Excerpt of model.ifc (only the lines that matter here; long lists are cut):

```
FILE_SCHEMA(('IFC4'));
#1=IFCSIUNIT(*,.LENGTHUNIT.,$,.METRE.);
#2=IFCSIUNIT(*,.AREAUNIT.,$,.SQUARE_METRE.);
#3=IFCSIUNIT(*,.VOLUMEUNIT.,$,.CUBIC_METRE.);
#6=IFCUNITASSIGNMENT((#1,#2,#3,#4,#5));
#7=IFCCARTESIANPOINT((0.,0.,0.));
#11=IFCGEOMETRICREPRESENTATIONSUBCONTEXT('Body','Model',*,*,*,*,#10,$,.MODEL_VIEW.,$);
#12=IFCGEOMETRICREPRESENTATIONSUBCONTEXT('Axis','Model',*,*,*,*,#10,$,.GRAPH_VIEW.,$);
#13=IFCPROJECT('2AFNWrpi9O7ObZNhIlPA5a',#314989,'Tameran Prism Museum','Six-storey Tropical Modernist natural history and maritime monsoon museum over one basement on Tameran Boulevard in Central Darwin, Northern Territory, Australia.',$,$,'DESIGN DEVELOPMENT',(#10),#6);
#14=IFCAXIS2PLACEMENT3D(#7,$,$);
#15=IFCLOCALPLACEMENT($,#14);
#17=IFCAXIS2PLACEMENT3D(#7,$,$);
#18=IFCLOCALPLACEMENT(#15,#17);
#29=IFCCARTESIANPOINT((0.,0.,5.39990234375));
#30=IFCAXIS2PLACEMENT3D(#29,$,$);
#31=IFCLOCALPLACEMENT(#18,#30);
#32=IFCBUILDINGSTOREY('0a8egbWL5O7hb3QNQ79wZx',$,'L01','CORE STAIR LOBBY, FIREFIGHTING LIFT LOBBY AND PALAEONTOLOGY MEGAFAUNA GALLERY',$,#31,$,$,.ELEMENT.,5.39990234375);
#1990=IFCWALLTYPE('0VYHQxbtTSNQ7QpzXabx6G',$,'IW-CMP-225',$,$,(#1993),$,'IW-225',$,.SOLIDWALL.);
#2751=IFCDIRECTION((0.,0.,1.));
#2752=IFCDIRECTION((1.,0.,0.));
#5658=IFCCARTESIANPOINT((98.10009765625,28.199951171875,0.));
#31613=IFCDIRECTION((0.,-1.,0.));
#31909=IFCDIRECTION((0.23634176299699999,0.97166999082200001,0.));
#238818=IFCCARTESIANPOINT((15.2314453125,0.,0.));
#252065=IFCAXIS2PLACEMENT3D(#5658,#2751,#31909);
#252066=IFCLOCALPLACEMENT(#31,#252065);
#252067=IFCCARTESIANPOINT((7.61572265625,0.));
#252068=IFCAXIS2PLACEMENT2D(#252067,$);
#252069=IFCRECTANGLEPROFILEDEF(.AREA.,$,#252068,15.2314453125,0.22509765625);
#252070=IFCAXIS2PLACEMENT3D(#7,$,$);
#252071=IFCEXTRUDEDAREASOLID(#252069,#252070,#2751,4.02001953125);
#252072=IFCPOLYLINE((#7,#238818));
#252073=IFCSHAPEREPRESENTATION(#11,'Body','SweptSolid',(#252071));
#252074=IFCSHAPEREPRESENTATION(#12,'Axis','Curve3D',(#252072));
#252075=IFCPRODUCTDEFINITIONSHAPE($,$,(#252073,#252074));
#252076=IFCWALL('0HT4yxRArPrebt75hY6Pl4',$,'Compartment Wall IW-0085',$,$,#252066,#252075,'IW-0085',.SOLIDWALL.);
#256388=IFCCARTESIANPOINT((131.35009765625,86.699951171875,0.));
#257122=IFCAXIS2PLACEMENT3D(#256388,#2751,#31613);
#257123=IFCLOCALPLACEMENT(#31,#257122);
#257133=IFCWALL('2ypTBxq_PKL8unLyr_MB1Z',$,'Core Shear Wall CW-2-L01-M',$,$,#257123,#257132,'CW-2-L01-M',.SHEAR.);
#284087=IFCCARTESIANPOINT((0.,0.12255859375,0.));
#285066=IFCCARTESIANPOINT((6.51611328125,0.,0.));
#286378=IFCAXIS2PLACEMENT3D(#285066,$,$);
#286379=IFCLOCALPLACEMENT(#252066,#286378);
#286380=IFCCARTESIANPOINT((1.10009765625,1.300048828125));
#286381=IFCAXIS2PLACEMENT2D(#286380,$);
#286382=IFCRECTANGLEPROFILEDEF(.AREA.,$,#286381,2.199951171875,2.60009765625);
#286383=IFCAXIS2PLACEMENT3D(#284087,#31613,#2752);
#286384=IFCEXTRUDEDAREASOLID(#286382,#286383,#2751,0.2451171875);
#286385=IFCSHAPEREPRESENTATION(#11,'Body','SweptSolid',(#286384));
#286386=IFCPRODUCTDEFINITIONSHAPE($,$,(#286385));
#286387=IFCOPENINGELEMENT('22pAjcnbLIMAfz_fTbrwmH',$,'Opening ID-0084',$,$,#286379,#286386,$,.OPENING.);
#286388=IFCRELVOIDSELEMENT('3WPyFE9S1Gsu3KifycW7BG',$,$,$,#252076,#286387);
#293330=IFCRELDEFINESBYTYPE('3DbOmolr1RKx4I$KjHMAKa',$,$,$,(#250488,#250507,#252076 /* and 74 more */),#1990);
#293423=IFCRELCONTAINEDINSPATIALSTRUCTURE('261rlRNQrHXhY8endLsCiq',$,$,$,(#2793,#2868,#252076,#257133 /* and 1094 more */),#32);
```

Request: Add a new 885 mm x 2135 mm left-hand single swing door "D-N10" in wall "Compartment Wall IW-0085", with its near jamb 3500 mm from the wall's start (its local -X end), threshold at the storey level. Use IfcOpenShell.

```python
import numpy as np
import ifcopenshell
import ifcopenshell.api.feature
import ifcopenshell.api.geometry
import ifcopenshell.api.root
import ifcopenshell.api.spatial
import ifcopenshell.geom
import ifcopenshell.util.element
import ifcopenshell.util.placement
import ifcopenshell.util.representation
import ifcopenshell.util.shape
import ifcopenshell.util.unit

model = ifcopenshell.open("model.ifc")
unit_scale = ifcopenshell.util.unit.calculate_unit_scale(model)
settings = ifcopenshell.geom.settings()


def volume(element):
    """Net volume in cubic metres, openings subtracted."""
    shape = ifcopenshell.geom.create_shape(settings, element)
    return ifcopenshell.util.shape.get_volume(shape.geometry)


wall = model.by_id(252076)
storey = ifcopenshell.util.element.get_container(wall, ifc_class="IfcBuildingStorey")
context = ifcopenshell.util.representation.get_context(model, "Model", "Body", "MODEL_VIEW")
before = volume(wall)

width, height, from_end, sill = 0.885, 2.135, 3.5, 0.0  # metres

# The wall runs along its own X axis, and the end named is its -X end.
wall_shape = ifcopenshell.geom.create_shape(settings, wall)
x, y, z = ifcopenshell.util.shape.get_vertices(wall_shape.geometry).T
start = x.min() + from_end
face, thickness = float(y.min()), float(y.max() - y.min())
wall_matrix = ifcopenshell.util.placement.get_local_placement(wall.ObjectPlacement)
level = ifcopenshell.util.placement.get_local_placement(storey.ObjectPlacement)[2, 3]


def in_wall(x, y):
    """Placement at x, y metres in the wall's axes, at sill height."""
    matrix = wall_matrix.copy()
    matrix[:, 3] = wall_matrix @ np.array([x / unit_scale, y / unit_scale, 0.0, 1.0])
    matrix[2, 3] = level + sill / unit_scale
    return matrix


# Opening: a box that overshoots both wall faces by 50 mm.
opening = ifcopenshell.api.root.create_entity(model, ifc_class="IfcOpeningElement", predefined_type="OPENING")
box = ifcopenshell.api.geometry.add_wall_representation(
    model, context=context, length=width, height=height, thickness=thickness + 0.1
)
ifcopenshell.api.geometry.assign_representation(model, product=opening, representation=box)
ifcopenshell.api.geometry.edit_object_placement(model, product=opening, matrix=in_wall(start, face - 0.05), is_si=False)
ifcopenshell.api.feature.add_feature(model, feature=opening, element=wall)

door = ifcopenshell.api.root.create_entity(model, ifc_class="IfcDoor", name="D-N10", predefined_type="DOOR")
door.OverallWidth, door.OverallHeight = width / unit_scale, height / unit_scale
door.OperationType = "SINGLE_SWING_LEFT"
body = ifcopenshell.api.geometry.add_door_representation(
    model,
    context=context,
    overall_width=door.OverallWidth,
    overall_height=door.OverallHeight,
    operation_type="SINGLE_SWING_LEFT",
    lining_properties={"LiningDepth": thickness / unit_scale, "ThresholdDepth": thickness / unit_scale},
)
ifcopenshell.api.geometry.assign_representation(model, product=door, representation=body)
ifcopenshell.api.spatial.assign_container(model, products=[door], relating_structure=storey)
ifcopenshell.api.feature.add_filling(model, opening=opening, element=door)

# The lining spans the wall, so the door starts at the wall face.
ifcopenshell.api.geometry.edit_object_placement(model, product=door, matrix=in_wall(start, face), is_si=False)

after = volume(wall)

print(f"wall volume {before:.3f} -> {after:.3f} m3")

model.write("model_updated.ifc")
```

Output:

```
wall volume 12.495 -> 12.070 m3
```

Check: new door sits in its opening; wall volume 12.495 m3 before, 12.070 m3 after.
